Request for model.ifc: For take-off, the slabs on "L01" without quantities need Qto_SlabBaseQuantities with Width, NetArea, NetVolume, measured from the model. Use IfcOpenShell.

First a look at what the model holds.

```python
import ifcopenshell
import ifcopenshell.util.element
import ifcopenshell.util.unit

model = ifcopenshell.open("model.ifc")
print(model.schema)
for unit_type in ("LENGTHUNIT", "AREAUNIT", "VOLUMEUNIT"):
    print(unit_type, ifcopenshell.util.unit.calculate_unit_scale(model, unit_type))
storey = next(s for s in model.by_type("IfcBuildingStorey") if s.Name == "L01")
slabs = [e for e in ifcopenshell.util.element.get_decomposition(storey) if e.is_a("IfcSlab")]
for e in sorted(slabs, key=lambda e: e.id()):
    print(e.id(), e.is_a(), e.Name, list(ifcopenshell.util.element.get_psets(e, qtos_only=True)), sep=" | ")
```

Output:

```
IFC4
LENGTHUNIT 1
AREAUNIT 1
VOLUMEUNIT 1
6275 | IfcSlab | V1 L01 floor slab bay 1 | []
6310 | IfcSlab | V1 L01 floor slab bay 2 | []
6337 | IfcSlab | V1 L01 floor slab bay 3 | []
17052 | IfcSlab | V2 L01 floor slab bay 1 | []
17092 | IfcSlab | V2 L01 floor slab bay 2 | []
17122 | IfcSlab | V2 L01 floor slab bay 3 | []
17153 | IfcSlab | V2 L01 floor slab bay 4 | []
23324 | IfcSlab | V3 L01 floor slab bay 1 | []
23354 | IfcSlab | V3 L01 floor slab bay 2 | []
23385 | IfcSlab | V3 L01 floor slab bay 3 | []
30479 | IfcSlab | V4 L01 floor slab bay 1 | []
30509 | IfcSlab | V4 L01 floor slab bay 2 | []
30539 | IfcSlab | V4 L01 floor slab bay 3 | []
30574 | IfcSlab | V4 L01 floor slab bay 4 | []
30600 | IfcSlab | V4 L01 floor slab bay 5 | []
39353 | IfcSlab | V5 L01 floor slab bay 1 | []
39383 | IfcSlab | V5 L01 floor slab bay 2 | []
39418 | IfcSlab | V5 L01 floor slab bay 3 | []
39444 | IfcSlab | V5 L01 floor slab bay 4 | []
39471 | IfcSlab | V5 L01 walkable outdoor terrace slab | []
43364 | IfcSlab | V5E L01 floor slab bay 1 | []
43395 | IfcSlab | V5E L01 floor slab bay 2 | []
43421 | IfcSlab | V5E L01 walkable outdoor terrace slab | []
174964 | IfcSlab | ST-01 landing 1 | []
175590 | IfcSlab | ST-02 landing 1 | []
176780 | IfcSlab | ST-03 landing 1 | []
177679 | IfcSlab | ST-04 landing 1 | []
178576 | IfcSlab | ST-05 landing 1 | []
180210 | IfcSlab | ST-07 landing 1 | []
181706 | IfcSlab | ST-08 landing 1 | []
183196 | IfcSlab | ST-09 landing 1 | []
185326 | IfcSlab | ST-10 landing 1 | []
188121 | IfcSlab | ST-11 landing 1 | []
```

```python
import ifcopenshell
import ifcopenshell.api.pset
import ifcopenshell.geom
import ifcopenshell.util.element
import ifcopenshell.util.shape
import ifcopenshell.util.unit

model = ifcopenshell.open("model.ifc")
unit_scale = ifcopenshell.util.unit.calculate_unit_scale(model)
area_scale = ifcopenshell.util.unit.calculate_unit_scale(model, "AREAUNIT")
volume_scale = ifcopenshell.util.unit.calculate_unit_scale(model, "VOLUMEUNIT")
settings = ifcopenshell.geom.settings()

storey = next(s for s in model.by_type("IfcBuildingStorey") if s.Name == "L01")
slabs = [e for e in ifcopenshell.util.element.get_decomposition(storey) if e.is_a("IfcSlab")]

for e in sorted(slabs, key=lambda e: e.id()):
    if ifcopenshell.util.element.get_psets(e, qtos_only=True, should_inherit=False):
        continue
    # Geometry comes back in metres, in the element's own axes.
    shape = ifcopenshell.geom.create_shape(settings, e)
    values = {
        "Width": ifcopenshell.util.shape.get_z(shape.geometry) / unit_scale,
        "NetArea": ifcopenshell.util.shape.get_footprint_area(shape.geometry) / area_scale,
        "NetVolume": ifcopenshell.util.shape.get_volume(shape.geometry) / volume_scale,
    }
    qto = ifcopenshell.api.pset.add_qto(model, product=e, name="Qto_SlabBaseQuantities")
    ifcopenshell.api.pset.edit_qto(model, qto=qto, properties=values)
    print(e.id(), {k: round(v, 3) for k, v in values.items()})

model.write("model_rev.ifc")
```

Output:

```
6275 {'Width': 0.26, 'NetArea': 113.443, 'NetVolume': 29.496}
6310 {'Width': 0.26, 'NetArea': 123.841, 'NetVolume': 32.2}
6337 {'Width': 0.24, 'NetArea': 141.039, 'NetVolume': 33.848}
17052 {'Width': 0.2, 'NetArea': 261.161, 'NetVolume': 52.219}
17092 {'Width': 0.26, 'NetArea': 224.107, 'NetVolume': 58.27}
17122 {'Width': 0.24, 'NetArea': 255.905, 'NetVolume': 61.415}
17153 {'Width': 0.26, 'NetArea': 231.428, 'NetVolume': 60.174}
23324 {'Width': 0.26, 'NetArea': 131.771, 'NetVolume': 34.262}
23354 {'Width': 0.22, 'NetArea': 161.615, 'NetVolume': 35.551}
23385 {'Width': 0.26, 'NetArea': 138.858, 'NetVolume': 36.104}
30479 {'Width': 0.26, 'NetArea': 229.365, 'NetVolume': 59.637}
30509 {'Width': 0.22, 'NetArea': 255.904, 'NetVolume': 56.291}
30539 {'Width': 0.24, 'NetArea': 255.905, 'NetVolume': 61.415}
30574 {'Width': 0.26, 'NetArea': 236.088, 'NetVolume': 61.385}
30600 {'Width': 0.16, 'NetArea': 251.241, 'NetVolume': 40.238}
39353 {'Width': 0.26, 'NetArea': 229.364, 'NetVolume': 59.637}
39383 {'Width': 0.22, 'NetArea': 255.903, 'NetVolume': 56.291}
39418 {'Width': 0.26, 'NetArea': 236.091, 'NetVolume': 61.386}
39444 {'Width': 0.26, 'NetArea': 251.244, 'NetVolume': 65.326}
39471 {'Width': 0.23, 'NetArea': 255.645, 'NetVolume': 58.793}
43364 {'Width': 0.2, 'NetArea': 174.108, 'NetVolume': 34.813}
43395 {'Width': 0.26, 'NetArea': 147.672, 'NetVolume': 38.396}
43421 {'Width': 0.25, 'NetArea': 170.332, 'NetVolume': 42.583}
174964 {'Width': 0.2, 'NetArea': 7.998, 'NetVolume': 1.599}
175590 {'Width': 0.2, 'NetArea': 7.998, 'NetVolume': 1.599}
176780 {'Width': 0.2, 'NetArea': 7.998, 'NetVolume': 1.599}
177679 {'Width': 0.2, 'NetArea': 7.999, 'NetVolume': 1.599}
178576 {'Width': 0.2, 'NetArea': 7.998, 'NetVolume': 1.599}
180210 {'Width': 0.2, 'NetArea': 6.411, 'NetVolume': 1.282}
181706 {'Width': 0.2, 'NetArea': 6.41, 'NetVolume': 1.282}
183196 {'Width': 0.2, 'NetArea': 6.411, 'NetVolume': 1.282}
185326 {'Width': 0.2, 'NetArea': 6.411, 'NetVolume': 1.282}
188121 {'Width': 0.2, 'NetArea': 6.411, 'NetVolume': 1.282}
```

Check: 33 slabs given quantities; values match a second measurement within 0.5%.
